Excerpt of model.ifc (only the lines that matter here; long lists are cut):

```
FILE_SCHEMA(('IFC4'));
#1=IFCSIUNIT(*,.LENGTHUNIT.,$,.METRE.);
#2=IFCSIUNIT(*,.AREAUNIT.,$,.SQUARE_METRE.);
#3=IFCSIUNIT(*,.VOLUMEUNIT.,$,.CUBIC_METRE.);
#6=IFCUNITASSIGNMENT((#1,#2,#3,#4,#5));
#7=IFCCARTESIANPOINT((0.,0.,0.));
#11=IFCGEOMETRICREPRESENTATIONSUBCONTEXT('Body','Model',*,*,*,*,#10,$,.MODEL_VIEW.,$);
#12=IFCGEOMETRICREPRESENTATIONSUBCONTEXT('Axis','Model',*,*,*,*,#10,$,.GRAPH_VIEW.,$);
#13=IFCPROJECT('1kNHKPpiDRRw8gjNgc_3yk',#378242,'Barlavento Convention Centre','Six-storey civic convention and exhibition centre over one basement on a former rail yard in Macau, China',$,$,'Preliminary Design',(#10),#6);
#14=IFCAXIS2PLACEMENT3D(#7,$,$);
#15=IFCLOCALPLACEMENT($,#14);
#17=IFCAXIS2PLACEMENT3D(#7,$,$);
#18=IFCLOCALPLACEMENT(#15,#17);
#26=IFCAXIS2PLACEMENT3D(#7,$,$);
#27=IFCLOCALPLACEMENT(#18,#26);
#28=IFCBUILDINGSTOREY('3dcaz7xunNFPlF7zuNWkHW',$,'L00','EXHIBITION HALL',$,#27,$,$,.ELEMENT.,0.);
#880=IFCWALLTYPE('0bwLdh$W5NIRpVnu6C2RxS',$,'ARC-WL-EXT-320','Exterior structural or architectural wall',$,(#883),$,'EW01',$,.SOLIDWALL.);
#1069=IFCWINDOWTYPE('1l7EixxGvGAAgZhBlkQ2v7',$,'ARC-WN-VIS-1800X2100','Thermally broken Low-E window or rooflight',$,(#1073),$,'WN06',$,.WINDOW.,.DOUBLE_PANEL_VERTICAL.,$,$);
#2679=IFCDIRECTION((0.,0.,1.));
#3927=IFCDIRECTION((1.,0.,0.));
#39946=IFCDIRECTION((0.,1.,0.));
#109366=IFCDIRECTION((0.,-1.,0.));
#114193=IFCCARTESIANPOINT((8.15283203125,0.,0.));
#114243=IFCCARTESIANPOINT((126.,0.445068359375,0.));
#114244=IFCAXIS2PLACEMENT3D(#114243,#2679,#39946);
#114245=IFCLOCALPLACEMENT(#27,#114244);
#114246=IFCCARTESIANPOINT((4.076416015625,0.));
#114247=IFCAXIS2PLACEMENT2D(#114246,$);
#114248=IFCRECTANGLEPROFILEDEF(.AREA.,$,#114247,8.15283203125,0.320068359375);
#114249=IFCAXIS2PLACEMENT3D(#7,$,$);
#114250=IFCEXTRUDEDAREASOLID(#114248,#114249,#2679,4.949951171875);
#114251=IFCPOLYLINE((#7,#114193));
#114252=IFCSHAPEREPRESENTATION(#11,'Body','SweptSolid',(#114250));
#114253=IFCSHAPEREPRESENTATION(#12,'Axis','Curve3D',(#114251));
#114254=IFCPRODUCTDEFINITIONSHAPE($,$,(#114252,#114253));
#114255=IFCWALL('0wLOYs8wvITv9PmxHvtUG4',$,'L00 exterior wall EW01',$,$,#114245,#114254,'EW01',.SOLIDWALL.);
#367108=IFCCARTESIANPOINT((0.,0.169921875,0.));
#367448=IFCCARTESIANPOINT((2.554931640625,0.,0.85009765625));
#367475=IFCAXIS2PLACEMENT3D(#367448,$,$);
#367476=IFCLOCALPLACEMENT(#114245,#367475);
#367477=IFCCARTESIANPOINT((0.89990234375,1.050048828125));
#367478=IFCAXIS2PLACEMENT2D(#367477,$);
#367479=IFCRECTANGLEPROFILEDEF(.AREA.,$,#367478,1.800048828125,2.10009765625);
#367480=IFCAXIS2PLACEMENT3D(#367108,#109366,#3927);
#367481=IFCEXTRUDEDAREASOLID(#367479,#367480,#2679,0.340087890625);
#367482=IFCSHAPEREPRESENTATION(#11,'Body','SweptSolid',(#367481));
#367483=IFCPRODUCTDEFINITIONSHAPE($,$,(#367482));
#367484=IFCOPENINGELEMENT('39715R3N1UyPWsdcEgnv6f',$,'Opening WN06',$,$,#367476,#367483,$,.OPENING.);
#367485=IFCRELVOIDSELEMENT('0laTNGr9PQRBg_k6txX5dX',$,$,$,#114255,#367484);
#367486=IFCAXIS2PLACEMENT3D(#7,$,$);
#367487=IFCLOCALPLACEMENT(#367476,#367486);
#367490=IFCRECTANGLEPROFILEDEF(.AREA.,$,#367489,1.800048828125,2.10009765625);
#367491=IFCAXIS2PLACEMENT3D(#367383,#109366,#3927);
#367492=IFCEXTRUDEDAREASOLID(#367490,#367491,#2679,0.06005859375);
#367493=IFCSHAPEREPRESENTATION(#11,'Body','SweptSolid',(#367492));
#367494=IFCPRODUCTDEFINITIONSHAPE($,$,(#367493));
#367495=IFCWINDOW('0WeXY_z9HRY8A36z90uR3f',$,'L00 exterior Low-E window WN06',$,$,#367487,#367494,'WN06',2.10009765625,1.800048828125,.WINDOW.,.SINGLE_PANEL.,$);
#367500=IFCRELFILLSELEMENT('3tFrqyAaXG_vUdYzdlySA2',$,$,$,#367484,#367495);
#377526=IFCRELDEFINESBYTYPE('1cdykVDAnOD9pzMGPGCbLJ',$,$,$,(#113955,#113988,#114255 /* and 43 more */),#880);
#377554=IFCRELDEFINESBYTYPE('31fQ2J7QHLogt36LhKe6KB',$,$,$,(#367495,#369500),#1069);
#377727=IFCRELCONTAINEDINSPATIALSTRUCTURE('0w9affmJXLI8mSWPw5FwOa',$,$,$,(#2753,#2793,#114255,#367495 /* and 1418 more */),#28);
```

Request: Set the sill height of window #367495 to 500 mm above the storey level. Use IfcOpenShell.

```python
import numpy as np
import ifcopenshell
import ifcopenshell.api.geometry
import ifcopenshell.geom
import ifcopenshell.util.element
import ifcopenshell.util.placement
import ifcopenshell.util.shape
import ifcopenshell.util.unit

model = ifcopenshell.open("model.ifc")
unit_scale = ifcopenshell.util.unit.calculate_unit_scale(model)

window = model.by_id(367495)
opening = window.FillsVoids[0].RelatingOpeningElement
storey = ifcopenshell.util.element.get_container(window, ifc_class="IfcBuildingStorey")
level = ifcopenshell.util.placement.get_local_placement(storey.ObjectPlacement)[2, 3]

# The opening's origin need not be at the sill, so measure its lowest point.
shape = ifcopenshell.geom.create_shape(ifcopenshell.geom.settings(), opening)
bottom = ifcopenshell.util.shape.get_shape_bottom_elevation(shape, shape.geometry) / unit_scale
dz = level + 0.5 - bottom

shift = np.array([0.0, 0.0, dz])
# The window is placed relative to its opening, so it follows when the opening moves.
matrix = ifcopenshell.util.placement.get_local_placement(opening.ObjectPlacement)
matrix[:3, 3] += shift
ifcopenshell.api.geometry.edit_object_placement(
    model, product=opening, matrix=matrix, is_si=False, should_transform_children=True
)

print(f"moved by {dz * unit_scale:+.3f} m")

model.write("model_rev.ifc")
```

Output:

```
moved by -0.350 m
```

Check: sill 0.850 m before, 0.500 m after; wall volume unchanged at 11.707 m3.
